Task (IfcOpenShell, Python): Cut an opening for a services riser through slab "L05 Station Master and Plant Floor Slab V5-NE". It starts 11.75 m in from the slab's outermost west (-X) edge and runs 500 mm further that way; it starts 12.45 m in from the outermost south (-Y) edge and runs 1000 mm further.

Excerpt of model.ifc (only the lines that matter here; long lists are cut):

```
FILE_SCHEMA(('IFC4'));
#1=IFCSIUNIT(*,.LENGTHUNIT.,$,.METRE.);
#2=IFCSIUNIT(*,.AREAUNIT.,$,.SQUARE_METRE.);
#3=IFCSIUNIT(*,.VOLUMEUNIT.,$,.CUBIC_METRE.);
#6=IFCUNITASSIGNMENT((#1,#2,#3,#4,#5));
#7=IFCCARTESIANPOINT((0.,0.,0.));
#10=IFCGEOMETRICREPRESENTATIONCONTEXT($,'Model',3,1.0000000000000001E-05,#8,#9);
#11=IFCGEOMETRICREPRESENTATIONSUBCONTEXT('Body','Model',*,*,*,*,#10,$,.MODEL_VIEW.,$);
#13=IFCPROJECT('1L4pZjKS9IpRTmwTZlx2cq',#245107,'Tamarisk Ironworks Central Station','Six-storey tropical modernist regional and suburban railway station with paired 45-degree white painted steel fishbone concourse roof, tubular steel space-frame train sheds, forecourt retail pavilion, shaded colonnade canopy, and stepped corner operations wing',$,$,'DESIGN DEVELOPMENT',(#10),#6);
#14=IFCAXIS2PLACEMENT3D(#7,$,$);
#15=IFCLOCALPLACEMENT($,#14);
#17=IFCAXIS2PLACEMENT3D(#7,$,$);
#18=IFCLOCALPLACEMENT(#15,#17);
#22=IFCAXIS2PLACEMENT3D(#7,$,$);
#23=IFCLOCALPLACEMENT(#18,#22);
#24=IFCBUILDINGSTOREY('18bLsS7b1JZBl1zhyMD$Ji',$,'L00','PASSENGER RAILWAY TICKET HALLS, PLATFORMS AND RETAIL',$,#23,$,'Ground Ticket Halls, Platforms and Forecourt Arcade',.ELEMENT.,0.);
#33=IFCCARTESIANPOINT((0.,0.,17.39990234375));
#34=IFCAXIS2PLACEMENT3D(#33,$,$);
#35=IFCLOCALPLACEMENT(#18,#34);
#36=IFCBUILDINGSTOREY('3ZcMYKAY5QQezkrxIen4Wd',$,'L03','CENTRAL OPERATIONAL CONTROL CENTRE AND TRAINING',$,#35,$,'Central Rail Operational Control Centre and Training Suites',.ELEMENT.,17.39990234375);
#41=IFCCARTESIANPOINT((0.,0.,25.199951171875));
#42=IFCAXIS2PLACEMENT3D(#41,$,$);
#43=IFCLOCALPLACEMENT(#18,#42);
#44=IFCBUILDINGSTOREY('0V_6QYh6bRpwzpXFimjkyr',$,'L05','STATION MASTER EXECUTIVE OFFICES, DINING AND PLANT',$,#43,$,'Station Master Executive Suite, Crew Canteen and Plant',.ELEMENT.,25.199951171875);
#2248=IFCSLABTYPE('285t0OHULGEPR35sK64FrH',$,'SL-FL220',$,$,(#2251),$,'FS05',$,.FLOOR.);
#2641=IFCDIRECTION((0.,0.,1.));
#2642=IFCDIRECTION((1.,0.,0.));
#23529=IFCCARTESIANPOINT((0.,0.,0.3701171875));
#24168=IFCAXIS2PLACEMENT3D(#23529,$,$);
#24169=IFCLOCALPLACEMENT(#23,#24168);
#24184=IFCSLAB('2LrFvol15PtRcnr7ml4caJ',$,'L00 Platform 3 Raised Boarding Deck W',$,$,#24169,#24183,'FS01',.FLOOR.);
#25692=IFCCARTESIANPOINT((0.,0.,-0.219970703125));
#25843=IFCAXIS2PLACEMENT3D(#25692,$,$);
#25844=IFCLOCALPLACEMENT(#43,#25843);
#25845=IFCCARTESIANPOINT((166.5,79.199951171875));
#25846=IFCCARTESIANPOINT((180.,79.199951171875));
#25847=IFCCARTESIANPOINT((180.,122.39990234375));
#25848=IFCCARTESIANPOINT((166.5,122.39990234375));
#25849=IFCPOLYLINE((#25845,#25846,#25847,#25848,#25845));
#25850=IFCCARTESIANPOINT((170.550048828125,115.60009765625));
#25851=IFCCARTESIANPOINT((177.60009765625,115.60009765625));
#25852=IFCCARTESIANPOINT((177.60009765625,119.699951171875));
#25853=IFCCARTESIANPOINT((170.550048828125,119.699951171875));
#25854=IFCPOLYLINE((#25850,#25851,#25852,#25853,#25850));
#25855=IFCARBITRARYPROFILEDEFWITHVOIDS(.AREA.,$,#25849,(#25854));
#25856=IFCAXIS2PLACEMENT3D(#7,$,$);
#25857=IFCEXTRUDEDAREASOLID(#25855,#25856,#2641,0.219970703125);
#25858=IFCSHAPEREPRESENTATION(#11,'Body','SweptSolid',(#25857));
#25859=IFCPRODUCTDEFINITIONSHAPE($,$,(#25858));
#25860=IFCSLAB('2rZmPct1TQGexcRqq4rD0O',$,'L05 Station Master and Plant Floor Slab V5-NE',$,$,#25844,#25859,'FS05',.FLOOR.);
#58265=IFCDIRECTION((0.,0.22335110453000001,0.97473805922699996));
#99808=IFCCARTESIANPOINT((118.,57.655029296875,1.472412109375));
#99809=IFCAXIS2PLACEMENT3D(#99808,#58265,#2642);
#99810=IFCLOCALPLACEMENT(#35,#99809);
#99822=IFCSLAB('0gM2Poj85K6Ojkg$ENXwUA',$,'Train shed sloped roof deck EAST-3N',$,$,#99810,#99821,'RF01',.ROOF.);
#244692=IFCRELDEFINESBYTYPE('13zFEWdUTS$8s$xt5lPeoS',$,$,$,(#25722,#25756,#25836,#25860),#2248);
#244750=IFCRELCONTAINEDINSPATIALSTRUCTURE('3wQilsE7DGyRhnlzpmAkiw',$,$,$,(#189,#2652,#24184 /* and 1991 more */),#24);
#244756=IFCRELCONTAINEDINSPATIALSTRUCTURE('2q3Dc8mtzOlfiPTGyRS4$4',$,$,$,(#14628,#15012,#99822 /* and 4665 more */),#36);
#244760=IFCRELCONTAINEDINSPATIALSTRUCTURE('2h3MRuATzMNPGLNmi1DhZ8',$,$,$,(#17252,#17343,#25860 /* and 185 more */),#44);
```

```python
import numpy as np
import ifcopenshell
import ifcopenshell.api.feature
import ifcopenshell.api.geometry
import ifcopenshell.api.root
import ifcopenshell.geom
import ifcopenshell.util.placement
import ifcopenshell.util.representation
import ifcopenshell.util.shape
import ifcopenshell.util.unit

model = ifcopenshell.open("model.ifc")
unit_scale = ifcopenshell.util.unit.calculate_unit_scale(model)
settings = ifcopenshell.geom.settings()


def volume(element):
    """Net volume in cubic metres, openings subtracted."""
    shape = ifcopenshell.geom.create_shape(settings, element)
    return ifcopenshell.util.shape.get_volume(shape.geometry)


slab = model.by_guid("2rZmPct1TQGexcRqq4rD0O")
before = volume(slab)

# Extent in the slab's own axes, in metres. The edges named are its -X and -Y sides.
slab_shape = ifcopenshell.geom.create_shape(settings, slab)
vertices = ifcopenshell.util.shape.get_vertices(slab_shape.geometry)
x_min, y_min, bottom = vertices.min(axis=0)
top = vertices[:, 2].max()

opening = ifcopenshell.api.root.create_entity(model, ifc_class="IfcOpeningElement", name="Services riser opening", predefined_type="OPENING")
context = ifcopenshell.util.representation.get_context(model, "Model", "Body", "MODEL_VIEW")
width, depth = 0.5, 1
outline = [(0.0, 0.0), (width, 0.0), (width, depth), (0.0, depth), (0.0, 0.0)]
# Overshoot both faces by 50 mm so the cut is clean.
shape = ifcopenshell.api.geometry.add_slab_representation(
    model, context=context, depth=top - bottom + 0.1, polyline=outline
)
ifcopenshell.api.geometry.assign_representation(model, product=opening, representation=shape)

matrix = ifcopenshell.util.placement.get_local_placement(slab.ObjectPlacement)
matrix[:, 3] = matrix @ np.append(np.array([x_min + 11.75, y_min + 12.45, bottom - 0.05]) / unit_scale, 1.0)
ifcopenshell.api.geometry.edit_object_placement(model, product=opening, matrix=matrix, is_si=False)
ifcopenshell.api.feature.add_feature(model, feature=opening, element=slab)

after = volume(slab)

print(f"slab volume {before:.3f} -> {after:.3f} m3")

model.write("model_v2.ifc")
```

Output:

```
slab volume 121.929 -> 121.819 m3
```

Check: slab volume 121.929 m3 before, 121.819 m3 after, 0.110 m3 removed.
